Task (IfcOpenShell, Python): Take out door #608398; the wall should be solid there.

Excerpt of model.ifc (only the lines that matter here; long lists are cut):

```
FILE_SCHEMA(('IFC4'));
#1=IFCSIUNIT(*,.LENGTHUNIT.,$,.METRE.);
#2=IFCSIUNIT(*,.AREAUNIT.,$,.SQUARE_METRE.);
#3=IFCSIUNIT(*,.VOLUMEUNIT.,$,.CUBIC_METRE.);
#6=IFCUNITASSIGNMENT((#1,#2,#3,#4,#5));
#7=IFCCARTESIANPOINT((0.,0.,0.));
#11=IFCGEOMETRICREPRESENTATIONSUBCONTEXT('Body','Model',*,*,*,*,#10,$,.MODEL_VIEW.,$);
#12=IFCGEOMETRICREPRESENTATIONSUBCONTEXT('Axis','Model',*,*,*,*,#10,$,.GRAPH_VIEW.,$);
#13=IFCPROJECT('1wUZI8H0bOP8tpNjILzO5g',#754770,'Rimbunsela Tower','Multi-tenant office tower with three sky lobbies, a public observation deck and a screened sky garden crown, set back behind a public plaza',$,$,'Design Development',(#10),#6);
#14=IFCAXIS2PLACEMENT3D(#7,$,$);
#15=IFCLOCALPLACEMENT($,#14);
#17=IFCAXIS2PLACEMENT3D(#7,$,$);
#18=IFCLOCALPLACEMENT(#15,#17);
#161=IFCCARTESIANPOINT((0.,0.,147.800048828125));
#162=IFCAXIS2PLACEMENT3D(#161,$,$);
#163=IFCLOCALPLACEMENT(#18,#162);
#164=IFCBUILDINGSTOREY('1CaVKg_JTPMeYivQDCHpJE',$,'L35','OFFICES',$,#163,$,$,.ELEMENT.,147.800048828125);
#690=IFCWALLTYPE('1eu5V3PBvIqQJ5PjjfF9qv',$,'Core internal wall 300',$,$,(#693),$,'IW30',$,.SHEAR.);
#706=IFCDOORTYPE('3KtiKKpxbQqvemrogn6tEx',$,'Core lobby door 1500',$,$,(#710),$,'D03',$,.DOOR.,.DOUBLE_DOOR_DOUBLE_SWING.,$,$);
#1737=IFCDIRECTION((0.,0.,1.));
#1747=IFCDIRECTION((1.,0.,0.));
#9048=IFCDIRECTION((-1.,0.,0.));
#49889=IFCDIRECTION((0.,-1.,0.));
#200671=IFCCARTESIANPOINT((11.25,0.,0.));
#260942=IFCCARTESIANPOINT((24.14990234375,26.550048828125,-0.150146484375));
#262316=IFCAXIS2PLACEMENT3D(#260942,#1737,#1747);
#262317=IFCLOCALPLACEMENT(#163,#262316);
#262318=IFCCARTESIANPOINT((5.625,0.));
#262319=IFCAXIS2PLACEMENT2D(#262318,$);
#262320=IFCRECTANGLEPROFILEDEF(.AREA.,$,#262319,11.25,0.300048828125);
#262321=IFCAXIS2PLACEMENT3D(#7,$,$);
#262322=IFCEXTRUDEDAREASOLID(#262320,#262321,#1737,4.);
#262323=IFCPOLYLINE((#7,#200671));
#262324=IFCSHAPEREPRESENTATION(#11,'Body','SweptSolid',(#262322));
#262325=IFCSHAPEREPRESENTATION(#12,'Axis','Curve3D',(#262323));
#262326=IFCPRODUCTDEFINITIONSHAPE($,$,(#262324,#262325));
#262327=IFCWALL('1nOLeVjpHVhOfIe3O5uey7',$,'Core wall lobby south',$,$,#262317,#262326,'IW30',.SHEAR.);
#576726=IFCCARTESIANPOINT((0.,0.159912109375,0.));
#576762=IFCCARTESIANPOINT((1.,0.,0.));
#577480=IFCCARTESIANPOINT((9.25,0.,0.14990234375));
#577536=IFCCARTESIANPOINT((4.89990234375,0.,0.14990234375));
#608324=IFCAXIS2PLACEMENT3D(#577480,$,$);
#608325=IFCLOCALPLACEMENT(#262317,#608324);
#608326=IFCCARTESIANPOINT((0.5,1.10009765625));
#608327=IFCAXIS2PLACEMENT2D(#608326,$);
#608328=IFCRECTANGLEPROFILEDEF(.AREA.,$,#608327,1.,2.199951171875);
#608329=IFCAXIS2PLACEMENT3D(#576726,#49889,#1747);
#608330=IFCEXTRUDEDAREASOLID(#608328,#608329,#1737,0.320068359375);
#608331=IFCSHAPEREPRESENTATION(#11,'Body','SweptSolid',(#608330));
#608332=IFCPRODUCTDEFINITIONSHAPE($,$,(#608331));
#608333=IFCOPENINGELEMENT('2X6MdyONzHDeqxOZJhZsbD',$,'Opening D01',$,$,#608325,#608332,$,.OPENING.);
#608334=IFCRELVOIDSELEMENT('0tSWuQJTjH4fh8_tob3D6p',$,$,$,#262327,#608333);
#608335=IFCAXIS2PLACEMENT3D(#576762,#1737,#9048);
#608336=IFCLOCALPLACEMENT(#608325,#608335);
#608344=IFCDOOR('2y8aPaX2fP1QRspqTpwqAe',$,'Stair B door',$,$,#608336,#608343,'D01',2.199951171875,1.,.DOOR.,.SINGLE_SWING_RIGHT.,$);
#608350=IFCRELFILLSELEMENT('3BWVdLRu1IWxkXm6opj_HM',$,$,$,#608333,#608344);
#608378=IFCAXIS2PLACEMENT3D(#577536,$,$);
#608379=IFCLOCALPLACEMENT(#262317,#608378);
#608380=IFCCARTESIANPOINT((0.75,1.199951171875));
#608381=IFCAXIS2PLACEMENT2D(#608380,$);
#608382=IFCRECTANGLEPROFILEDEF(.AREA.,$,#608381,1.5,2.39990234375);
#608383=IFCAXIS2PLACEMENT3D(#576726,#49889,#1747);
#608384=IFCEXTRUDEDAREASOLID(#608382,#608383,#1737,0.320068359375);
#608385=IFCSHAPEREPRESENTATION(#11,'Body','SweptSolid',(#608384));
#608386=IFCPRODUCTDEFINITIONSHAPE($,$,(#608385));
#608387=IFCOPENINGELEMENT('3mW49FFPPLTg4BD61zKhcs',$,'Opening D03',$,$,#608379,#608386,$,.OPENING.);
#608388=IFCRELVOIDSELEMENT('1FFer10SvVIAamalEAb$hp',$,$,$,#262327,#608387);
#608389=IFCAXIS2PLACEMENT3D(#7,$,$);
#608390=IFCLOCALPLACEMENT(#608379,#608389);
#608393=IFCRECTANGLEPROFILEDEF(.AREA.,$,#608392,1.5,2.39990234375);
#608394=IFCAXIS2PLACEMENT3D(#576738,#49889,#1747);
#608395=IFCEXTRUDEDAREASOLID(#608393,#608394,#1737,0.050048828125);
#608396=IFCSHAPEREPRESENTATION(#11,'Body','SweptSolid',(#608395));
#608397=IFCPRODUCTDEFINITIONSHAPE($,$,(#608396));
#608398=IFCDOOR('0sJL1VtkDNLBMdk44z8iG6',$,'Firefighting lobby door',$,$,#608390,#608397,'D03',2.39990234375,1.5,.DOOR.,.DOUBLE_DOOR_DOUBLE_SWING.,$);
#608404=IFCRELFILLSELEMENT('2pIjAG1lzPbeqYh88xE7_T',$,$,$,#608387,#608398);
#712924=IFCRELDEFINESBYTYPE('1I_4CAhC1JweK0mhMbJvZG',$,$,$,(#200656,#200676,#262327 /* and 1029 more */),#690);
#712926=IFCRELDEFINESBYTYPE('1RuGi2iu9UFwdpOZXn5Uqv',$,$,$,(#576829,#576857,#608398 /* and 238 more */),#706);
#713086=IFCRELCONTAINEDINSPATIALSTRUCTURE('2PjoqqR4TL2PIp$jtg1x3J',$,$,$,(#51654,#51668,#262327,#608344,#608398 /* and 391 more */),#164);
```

```python
import ifcopenshell
import ifcopenshell.api.feature
import ifcopenshell.api.root
import ifcopenshell.geom
import ifcopenshell.util.shape

model = ifcopenshell.open("model.ifc")
settings = ifcopenshell.geom.settings()


def volume(element):
    """Net volume in cubic metres, openings subtracted."""
    shape = ifcopenshell.geom.create_shape(settings, element)
    return ifcopenshell.util.shape.get_volume(shape.geometry)


door = model.by_guid("0sJL1VtkDNLBMdk44z8iG6")
opening = door.FillsVoids[0].RelatingOpeningElement
wall = opening.VoidsElements[0].RelatingBuildingElement
before = volume(wall)

ifcopenshell.api.root.remove_product(model, product=door)
ifcopenshell.api.feature.remove_feature(model, feature=opening)

after = volume(wall)

print(f"wall volume {before:.3f} -> {after:.3f} m3")

model.write("model-out.ifc")
```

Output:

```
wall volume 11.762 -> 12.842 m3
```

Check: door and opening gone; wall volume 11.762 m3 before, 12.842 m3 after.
